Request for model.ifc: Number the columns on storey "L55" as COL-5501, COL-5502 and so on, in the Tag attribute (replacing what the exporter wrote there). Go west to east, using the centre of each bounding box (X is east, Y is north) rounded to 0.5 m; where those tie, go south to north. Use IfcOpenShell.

First a look at what the model holds.

```python
import ifcopenshell
import ifcopenshell.util.element
import ifcopenshell.util.placement

model = ifcopenshell.open("model.ifc")
print(model.schema)
storey = next(s for s in model.by_type("IfcBuildingStorey") if s.Name == "L55")
columns = [e for e in ifcopenshell.util.element.get_decomposition(storey) if e.is_a("IfcColumn")]
for e in sorted(columns, key=lambda e: e.id()):
    origin = ifcopenshell.util.placement.get_local_placement(e.ObjectPlacement)[:3, 3]
    print(e.id(), e.Tag, e.Name, origin.round(2) + 0.0, sep=" | ")
```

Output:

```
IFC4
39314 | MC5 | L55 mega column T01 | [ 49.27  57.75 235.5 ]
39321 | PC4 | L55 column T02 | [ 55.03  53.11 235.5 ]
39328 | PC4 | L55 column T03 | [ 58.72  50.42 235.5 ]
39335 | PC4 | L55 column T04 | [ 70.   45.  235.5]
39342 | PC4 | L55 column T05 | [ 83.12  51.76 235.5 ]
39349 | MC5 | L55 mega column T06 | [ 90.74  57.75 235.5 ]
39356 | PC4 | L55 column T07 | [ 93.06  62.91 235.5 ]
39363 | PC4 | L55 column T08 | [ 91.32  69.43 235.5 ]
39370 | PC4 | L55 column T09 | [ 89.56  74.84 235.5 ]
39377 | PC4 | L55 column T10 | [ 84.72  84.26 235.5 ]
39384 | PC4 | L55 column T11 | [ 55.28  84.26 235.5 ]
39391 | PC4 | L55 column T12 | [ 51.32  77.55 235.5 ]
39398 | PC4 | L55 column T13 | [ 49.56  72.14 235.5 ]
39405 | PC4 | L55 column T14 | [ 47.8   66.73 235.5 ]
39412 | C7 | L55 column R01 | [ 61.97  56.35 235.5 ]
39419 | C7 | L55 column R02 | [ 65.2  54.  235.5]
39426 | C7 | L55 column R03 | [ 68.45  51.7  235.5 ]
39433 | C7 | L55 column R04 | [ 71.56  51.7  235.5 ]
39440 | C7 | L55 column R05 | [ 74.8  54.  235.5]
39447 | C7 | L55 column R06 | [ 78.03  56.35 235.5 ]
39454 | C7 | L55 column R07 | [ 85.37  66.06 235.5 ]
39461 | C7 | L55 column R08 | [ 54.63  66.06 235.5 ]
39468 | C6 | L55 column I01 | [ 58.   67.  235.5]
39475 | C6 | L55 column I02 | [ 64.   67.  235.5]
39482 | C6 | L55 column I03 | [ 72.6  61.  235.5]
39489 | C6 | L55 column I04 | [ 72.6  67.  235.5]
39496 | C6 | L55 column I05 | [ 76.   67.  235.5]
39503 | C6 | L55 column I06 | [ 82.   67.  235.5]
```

```python
import ifcopenshell
import ifcopenshell.geom
import ifcopenshell.util.element
import ifcopenshell.util.shape

model = ifcopenshell.open("model.ifc")
settings = ifcopenshell.geom.settings()
settings.set("use-world-coords", True)


def centre(element):
    shape = ifcopenshell.geom.create_shape(settings, element)
    return ifcopenshell.util.shape.get_bbox_centroid(shape.geometry)


storey = next(s for s in model.by_type("IfcBuildingStorey") if s.Name == "L55")
columns = [e for e in ifcopenshell.util.element.get_decomposition(storey) if e.is_a("IfcColumn")]

# Insertion points can sit at a corner or the storey origin, so sort by the geometry (in metres).
centres = {e: centre(e) for e in columns}
columns.sort(key=lambda e: (round(centres[e][0] / 0.5), centres[e][1]))

for i, e in enumerate(columns, start=1):
    number = f"COL-55{i:02d}"
    e.Tag = number
    print(e.id(), number)

model.write("model-out.ifc")
```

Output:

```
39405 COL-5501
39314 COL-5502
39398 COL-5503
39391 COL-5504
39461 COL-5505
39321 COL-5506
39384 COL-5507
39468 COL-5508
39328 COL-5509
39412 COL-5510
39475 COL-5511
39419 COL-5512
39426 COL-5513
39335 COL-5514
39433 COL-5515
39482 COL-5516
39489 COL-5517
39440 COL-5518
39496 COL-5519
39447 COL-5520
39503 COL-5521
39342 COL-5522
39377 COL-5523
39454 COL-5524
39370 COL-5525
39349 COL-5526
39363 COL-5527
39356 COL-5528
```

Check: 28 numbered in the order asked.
